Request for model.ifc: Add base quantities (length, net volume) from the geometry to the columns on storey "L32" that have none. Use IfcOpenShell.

First a look at what the model holds.

```python
import ifcopenshell
import ifcopenshell.util.element
import ifcopenshell.util.unit

model = ifcopenshell.open("model.ifc")
print(model.schema)
for unit_type in ("LENGTHUNIT", "AREAUNIT", "VOLUMEUNIT"):
    print(unit_type, ifcopenshell.util.unit.calculate_unit_scale(model, unit_type))
storey = next(s for s in model.by_type("IfcBuildingStorey") if s.Name == "L32")
columns = [e for e in ifcopenshell.util.element.get_decomposition(storey) if e.is_a("IfcColumn")]
for e in sorted(columns, key=lambda e: e.id()):
    print(e.id(), e.is_a(), e.Name, list(ifcopenshell.util.element.get_psets(e, qtos_only=True)), sep=" | ")
```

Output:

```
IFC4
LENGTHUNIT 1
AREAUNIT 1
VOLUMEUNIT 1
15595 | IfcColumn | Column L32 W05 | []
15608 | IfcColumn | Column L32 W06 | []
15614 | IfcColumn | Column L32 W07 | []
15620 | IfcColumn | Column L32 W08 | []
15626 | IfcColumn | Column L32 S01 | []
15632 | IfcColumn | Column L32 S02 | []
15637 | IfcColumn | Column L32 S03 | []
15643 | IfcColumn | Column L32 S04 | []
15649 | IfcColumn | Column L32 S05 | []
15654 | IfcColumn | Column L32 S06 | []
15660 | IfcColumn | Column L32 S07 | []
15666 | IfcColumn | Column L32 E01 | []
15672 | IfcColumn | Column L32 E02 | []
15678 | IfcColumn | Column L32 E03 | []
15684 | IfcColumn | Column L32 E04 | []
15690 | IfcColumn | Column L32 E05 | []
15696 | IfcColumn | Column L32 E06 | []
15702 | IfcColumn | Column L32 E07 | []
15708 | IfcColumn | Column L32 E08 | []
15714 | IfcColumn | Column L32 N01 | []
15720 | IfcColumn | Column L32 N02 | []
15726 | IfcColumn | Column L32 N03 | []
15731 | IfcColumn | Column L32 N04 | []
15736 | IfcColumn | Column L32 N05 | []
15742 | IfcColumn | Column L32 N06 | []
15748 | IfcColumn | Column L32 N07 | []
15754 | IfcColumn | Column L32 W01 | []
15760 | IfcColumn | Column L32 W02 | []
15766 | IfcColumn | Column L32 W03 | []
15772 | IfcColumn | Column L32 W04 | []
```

```python
import ifcopenshell
import ifcopenshell.api.pset
import ifcopenshell.geom
import ifcopenshell.util.element
import ifcopenshell.util.shape
import ifcopenshell.util.unit

model = ifcopenshell.open("model.ifc")
unit_scale = ifcopenshell.util.unit.calculate_unit_scale(model)
volume_scale = ifcopenshell.util.unit.calculate_unit_scale(model, "VOLUMEUNIT")
settings = ifcopenshell.geom.settings()

storey = next(s for s in model.by_type("IfcBuildingStorey") if s.Name == "L32")
columns = [e for e in ifcopenshell.util.element.get_decomposition(storey) if e.is_a("IfcColumn")]

for e in sorted(columns, key=lambda e: e.id()):
    if ifcopenshell.util.element.get_psets(e, qtos_only=True, should_inherit=False):
        continue
    # Geometry comes back in metres, in the element's own axes.
    shape = ifcopenshell.geom.create_shape(settings, e)
    values = {
        "Length": ifcopenshell.util.shape.get_z(shape.geometry) / unit_scale,
        "NetVolume": ifcopenshell.util.shape.get_volume(shape.geometry) / volume_scale,
    }
    qto = ifcopenshell.api.pset.add_qto(model, product=e, name="Qto_ColumnBaseQuantities")
    ifcopenshell.api.pset.edit_qto(model, qto=qto, properties=values)
    print(e.id(), {k: round(v, 3) for k, v in values.items()})

model.write("model_edited.ifc")
```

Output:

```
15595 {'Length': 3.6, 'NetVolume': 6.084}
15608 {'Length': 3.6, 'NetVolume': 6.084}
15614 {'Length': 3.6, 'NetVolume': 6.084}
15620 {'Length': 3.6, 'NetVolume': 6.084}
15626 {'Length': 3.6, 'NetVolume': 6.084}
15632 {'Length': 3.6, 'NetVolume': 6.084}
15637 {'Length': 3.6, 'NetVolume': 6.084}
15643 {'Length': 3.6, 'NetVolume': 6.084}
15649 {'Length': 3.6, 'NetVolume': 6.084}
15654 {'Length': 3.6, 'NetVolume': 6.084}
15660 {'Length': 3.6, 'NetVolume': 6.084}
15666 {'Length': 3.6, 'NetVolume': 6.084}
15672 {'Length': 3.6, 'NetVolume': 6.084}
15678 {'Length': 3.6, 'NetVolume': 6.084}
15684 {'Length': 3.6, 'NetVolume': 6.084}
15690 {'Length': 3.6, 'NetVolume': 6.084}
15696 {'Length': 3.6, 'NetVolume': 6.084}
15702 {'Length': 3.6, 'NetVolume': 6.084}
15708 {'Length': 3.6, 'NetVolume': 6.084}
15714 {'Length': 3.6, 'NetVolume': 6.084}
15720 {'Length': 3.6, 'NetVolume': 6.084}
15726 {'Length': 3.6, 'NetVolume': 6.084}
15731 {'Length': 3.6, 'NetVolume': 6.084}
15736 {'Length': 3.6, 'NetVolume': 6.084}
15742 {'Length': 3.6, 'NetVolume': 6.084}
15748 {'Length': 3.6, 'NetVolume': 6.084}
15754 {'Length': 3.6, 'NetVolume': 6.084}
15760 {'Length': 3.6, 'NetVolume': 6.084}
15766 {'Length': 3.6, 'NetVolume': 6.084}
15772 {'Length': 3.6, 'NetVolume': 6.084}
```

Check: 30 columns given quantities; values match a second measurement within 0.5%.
